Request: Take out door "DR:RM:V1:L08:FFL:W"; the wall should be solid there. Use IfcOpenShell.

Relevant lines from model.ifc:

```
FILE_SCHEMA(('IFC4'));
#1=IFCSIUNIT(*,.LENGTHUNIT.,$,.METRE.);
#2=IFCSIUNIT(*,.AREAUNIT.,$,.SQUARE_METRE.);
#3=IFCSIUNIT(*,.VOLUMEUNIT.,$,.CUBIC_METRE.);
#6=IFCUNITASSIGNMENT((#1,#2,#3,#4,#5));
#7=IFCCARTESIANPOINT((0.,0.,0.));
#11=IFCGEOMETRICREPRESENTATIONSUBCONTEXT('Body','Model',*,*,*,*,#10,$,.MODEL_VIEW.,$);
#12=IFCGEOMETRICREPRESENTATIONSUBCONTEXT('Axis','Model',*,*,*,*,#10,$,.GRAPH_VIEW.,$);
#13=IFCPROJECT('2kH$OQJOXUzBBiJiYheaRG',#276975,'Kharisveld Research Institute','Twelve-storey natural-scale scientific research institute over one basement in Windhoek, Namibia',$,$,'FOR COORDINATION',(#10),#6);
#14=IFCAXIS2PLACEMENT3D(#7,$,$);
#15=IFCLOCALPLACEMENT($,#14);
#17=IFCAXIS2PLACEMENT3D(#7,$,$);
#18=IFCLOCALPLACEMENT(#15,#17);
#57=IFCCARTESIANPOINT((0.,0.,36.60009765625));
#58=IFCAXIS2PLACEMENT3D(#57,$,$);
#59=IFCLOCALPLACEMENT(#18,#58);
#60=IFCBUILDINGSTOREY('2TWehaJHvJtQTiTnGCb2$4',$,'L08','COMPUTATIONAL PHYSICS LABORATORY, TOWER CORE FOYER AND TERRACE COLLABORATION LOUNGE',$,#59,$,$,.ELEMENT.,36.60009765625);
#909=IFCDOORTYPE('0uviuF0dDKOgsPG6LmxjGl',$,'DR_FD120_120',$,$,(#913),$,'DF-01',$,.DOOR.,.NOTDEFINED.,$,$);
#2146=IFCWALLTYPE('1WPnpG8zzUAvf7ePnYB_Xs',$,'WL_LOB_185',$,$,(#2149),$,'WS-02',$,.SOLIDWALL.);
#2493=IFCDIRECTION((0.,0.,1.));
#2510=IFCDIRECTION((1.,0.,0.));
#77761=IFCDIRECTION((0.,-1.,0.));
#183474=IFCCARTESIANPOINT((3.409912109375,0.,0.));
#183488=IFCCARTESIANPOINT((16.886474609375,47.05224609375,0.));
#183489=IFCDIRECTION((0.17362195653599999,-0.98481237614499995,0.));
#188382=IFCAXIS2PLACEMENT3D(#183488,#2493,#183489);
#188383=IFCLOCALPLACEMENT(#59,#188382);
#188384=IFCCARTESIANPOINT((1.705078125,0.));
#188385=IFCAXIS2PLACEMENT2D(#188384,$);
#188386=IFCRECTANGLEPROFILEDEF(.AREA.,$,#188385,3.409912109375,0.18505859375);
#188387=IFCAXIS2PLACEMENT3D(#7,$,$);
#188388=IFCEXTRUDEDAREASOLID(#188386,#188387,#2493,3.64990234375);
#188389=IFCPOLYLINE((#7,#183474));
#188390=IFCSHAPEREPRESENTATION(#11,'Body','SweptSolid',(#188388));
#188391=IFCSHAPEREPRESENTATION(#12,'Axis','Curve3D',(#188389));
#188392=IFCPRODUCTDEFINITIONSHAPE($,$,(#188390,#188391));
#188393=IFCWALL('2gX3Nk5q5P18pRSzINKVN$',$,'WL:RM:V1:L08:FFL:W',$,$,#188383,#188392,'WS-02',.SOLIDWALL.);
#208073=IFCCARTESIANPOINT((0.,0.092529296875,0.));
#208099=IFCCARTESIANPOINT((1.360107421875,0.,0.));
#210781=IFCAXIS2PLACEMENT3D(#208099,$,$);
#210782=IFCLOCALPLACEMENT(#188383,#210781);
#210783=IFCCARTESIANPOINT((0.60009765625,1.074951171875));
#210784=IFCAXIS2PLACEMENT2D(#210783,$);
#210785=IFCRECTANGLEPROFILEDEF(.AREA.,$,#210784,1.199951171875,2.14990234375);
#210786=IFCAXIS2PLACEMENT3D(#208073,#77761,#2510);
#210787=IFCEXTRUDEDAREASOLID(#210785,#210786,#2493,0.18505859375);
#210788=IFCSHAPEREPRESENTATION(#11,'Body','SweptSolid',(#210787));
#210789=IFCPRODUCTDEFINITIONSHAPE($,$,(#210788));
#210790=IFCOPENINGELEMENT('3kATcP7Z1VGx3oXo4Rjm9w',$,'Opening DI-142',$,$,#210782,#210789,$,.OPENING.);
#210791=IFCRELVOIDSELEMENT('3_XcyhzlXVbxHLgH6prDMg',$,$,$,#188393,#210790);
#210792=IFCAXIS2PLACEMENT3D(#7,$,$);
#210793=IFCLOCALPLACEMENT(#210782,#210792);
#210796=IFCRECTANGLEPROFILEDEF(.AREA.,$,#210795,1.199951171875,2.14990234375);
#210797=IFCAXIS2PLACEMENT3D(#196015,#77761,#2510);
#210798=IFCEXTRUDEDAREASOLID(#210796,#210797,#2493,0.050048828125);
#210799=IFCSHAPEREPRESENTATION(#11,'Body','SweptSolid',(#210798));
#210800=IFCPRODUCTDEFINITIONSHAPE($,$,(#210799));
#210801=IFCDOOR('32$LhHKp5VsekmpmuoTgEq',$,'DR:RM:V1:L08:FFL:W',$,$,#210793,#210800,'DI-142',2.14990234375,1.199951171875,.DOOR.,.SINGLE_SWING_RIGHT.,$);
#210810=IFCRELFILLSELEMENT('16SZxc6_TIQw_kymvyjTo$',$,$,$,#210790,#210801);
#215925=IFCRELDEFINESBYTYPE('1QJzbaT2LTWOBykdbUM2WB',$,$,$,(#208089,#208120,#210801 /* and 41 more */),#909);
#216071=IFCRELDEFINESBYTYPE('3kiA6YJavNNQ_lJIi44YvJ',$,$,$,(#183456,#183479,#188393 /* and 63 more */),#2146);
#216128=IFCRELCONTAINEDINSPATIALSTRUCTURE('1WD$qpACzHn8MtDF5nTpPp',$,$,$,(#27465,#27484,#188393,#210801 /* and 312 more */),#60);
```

```python
import ifcopenshell
import ifcopenshell.api.feature
import ifcopenshell.api.root
import ifcopenshell.geom
import ifcopenshell.util.shape

model = ifcopenshell.open("model.ifc")
settings = ifcopenshell.geom.settings()


def volume(element):
    """Net volume in cubic metres, openings subtracted."""
    shape = ifcopenshell.geom.create_shape(settings, element)
    return ifcopenshell.util.shape.get_volume(shape.geometry)


door = model.by_guid("32$LhHKp5VsekmpmuoTgEq")
opening = door.FillsVoids[0].RelatingOpeningElement
wall = opening.VoidsElements[0].RelatingBuildingElement
before = volume(wall)

ifcopenshell.api.root.remove_product(model, product=door)
ifcopenshell.api.feature.remove_feature(model, feature=opening)

after = volume(wall)

print(f"wall volume {before:.3f} -> {after:.3f} m3")

model.write("model_updated.ifc")
```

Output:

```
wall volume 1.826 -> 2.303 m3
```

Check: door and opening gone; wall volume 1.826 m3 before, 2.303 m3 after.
